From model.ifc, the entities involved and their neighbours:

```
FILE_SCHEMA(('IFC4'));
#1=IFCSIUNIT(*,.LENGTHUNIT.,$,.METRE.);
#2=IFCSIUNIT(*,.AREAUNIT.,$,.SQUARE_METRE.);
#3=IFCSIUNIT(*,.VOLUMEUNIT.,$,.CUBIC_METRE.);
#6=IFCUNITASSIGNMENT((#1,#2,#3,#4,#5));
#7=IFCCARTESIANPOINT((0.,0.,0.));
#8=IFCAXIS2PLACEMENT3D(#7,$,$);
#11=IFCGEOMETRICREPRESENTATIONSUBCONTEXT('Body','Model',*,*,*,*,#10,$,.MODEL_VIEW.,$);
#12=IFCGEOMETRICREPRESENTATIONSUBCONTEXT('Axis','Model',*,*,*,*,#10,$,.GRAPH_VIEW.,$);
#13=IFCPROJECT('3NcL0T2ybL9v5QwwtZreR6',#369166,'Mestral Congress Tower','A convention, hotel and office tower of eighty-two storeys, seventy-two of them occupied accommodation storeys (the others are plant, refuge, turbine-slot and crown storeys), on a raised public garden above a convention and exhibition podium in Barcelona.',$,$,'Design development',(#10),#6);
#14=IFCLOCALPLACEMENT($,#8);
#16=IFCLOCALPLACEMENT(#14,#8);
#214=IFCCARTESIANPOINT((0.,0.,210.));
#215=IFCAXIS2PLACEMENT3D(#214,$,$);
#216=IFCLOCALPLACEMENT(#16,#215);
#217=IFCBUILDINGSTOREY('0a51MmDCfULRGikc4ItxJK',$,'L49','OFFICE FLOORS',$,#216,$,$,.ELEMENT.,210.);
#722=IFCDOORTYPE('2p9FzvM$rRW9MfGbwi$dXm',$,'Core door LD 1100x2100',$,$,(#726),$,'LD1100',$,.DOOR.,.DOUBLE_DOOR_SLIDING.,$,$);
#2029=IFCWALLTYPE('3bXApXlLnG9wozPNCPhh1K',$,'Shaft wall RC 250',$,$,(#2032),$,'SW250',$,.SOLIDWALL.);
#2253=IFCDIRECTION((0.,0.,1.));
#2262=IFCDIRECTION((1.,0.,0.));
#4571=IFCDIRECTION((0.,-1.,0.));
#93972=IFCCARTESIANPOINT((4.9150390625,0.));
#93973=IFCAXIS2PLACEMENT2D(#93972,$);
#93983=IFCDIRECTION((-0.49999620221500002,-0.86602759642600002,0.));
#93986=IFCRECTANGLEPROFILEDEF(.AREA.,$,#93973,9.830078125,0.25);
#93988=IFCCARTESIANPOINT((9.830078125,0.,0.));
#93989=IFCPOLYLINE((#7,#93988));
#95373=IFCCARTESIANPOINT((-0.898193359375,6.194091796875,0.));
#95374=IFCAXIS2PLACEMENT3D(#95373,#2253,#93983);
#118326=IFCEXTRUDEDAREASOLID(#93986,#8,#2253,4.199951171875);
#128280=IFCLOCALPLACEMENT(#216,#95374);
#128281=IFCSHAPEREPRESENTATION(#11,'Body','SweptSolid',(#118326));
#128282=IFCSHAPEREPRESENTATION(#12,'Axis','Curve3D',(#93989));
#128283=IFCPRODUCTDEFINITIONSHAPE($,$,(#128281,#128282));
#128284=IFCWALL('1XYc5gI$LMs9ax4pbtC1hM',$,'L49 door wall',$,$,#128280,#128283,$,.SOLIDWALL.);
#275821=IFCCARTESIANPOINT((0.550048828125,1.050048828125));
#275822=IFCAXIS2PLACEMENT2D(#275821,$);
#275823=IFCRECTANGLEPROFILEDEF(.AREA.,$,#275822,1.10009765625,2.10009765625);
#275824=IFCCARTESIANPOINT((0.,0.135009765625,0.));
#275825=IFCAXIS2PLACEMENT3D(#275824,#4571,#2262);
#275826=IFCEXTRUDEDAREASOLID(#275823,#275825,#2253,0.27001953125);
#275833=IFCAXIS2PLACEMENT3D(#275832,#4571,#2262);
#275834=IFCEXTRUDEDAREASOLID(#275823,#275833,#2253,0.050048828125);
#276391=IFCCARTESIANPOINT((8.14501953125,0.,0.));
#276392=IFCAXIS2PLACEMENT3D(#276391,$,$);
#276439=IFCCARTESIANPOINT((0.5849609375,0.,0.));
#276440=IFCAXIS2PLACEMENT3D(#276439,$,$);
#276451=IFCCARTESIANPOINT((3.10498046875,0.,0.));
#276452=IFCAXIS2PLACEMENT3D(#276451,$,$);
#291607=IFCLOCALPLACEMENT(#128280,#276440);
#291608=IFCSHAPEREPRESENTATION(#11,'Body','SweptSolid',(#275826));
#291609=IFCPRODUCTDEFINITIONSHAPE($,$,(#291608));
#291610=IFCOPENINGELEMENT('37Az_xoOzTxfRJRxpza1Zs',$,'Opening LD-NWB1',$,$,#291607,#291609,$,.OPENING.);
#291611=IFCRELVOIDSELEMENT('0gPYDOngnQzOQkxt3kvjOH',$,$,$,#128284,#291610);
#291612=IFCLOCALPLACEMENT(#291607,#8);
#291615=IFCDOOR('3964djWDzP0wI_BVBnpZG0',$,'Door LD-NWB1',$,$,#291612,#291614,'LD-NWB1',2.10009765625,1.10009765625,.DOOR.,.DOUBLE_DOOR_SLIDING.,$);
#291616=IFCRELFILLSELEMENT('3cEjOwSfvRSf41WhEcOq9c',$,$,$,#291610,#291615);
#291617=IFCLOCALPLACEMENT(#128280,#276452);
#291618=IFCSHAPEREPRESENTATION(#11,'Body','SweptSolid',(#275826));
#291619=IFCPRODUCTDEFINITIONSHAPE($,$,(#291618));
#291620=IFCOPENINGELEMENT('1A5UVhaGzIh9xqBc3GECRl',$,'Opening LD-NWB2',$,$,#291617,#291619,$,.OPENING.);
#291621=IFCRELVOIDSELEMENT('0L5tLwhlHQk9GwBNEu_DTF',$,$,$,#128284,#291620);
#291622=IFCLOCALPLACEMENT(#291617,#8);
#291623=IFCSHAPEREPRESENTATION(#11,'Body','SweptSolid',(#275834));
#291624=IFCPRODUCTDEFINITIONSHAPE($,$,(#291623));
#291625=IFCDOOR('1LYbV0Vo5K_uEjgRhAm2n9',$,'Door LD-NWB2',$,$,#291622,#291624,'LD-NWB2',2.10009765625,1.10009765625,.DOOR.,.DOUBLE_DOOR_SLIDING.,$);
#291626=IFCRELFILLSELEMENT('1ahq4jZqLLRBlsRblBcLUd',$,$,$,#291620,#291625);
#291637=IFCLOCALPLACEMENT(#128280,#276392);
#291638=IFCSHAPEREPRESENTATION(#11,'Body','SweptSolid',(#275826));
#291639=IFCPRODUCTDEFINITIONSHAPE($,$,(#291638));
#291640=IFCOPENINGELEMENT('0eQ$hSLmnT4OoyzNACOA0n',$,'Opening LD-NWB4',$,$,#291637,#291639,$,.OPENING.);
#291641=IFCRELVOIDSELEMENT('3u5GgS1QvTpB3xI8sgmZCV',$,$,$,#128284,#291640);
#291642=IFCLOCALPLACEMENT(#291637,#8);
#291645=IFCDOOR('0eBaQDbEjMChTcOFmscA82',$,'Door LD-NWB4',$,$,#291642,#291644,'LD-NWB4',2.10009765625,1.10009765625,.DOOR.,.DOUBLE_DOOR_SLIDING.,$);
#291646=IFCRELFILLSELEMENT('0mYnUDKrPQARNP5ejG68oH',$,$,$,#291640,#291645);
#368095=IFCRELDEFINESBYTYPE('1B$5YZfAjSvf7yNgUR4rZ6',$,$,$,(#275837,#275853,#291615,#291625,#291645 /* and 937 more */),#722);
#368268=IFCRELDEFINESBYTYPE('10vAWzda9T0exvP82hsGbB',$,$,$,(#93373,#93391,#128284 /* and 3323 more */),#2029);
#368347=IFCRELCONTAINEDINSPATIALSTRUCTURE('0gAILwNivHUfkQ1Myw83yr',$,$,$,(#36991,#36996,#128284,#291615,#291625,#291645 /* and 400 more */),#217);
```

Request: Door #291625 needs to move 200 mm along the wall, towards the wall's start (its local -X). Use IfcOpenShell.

```python
import ifcopenshell
import ifcopenshell.api.geometry
import ifcopenshell.util.placement

model = ifcopenshell.open("model.ifc")

door = model.by_guid("1LYbV0Vo5K_uEjgRhAm2n9")
opening = door.FillsVoids[0].RelatingOpeningElement
wall = opening.VoidsElements[0].RelatingBuildingElement

wall_matrix = ifcopenshell.util.placement.get_local_placement(wall.ObjectPlacement)
shift = wall_matrix[:3, 0] * -0.2
before = ifcopenshell.util.placement.get_local_placement(door.ObjectPlacement)[:3, 3].copy()

# The door is placed relative to its opening, so it follows when the opening moves.
matrix = ifcopenshell.util.placement.get_local_placement(opening.ObjectPlacement)
matrix[:3, 3] += shift
ifcopenshell.api.geometry.edit_object_placement(
    model, product=opening, matrix=matrix, is_si=False, should_transform_children=True
)

after = ifcopenshell.util.placement.get_local_placement(door.ObjectPlacement)[:3, 3]
print("door moved by", (after - before).round(3) + 0.0)

model.write("model_v2.ifc")
```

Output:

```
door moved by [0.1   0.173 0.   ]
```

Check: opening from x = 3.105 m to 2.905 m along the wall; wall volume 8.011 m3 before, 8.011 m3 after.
